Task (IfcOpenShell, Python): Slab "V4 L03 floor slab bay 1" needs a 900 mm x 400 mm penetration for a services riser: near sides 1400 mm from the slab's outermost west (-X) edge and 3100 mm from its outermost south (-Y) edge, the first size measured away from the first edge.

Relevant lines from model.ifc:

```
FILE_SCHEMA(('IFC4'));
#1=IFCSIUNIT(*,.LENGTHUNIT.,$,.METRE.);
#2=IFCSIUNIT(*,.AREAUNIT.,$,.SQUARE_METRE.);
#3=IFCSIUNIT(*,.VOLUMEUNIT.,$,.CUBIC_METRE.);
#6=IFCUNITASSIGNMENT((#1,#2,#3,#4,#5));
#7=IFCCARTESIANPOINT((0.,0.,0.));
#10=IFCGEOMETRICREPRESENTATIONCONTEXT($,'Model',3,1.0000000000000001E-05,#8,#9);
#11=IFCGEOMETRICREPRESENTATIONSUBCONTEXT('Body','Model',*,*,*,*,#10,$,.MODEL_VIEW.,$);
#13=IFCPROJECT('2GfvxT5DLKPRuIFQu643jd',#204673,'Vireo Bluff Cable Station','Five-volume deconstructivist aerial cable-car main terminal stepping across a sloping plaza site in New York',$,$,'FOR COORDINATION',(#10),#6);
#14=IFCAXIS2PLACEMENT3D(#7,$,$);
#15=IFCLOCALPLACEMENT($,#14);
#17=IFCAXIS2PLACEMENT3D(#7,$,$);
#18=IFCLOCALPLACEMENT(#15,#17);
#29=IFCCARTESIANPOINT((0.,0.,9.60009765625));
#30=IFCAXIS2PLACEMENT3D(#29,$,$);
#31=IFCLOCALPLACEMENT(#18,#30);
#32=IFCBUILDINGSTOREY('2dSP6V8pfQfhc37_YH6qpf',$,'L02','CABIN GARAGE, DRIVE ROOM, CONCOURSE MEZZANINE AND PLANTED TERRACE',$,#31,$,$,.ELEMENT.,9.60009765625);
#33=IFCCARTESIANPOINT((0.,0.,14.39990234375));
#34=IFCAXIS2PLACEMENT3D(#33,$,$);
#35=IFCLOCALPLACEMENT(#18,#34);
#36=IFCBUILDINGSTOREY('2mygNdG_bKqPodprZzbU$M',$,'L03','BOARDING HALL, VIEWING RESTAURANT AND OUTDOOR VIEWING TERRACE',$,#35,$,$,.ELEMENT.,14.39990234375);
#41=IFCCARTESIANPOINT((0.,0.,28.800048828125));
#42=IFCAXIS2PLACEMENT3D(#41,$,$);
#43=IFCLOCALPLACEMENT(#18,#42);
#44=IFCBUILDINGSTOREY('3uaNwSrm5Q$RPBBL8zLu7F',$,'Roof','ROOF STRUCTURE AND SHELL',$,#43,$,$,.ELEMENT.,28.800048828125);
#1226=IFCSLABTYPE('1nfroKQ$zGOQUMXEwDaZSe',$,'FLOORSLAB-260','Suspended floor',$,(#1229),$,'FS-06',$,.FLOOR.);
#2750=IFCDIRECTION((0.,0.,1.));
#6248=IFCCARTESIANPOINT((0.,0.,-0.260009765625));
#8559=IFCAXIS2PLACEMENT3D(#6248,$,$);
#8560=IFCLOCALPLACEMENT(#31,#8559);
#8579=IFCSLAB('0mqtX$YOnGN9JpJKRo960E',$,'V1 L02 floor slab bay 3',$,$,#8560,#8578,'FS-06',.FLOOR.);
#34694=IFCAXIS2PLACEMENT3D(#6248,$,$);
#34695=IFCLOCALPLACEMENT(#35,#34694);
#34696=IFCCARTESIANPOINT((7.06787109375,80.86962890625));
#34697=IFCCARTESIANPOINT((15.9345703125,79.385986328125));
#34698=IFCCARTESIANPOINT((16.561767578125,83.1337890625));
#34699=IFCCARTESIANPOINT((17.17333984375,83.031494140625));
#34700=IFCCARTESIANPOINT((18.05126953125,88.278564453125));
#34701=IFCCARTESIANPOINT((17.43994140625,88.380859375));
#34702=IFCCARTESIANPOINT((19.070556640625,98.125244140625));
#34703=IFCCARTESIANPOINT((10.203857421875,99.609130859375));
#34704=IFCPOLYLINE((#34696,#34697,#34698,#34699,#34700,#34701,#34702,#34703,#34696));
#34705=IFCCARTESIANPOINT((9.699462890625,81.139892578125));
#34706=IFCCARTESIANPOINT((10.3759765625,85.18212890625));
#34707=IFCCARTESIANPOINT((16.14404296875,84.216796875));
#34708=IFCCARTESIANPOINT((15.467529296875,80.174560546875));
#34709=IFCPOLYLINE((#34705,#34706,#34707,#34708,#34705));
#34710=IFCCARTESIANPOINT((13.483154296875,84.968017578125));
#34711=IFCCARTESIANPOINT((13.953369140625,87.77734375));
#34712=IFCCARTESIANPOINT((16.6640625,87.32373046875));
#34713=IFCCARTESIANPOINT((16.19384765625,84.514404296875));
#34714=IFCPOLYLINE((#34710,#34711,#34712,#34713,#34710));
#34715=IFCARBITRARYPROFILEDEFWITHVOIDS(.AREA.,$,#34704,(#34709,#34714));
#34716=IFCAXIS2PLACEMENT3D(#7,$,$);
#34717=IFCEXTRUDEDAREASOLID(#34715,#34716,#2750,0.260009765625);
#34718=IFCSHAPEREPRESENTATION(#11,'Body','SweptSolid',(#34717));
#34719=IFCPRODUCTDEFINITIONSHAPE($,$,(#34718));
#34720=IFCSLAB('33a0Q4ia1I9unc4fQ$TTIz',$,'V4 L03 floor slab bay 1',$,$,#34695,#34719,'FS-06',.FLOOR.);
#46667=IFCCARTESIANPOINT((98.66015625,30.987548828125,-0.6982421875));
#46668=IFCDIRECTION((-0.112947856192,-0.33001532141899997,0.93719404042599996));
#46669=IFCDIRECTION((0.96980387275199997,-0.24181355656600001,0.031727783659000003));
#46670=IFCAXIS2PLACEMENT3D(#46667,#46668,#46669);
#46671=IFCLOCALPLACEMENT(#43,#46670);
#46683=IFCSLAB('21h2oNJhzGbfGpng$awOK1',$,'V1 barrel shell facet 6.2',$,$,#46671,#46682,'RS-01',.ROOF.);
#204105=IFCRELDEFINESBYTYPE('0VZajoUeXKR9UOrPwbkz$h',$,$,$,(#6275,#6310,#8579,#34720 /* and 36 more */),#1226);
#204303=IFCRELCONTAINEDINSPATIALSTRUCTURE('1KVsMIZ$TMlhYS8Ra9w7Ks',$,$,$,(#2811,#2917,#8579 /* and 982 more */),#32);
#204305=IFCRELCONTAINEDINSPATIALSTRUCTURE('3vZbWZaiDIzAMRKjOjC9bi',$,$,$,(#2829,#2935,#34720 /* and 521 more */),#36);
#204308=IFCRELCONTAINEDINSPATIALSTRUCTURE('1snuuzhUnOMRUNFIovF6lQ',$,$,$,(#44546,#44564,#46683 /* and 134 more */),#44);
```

```python
import numpy as np
import ifcopenshell
import ifcopenshell.api.feature
import ifcopenshell.api.geometry
import ifcopenshell.api.root
import ifcopenshell.geom
import ifcopenshell.util.placement
import ifcopenshell.util.representation
import ifcopenshell.util.shape
import ifcopenshell.util.unit

model = ifcopenshell.open("model.ifc")
unit_scale = ifcopenshell.util.unit.calculate_unit_scale(model)
settings = ifcopenshell.geom.settings()


def volume(element):
    """Net volume in cubic metres, openings subtracted."""
    shape = ifcopenshell.geom.create_shape(settings, element)
    return ifcopenshell.util.shape.get_volume(shape.geometry)


slab = model.by_guid("33a0Q4ia1I9unc4fQ$TTIz")
before = volume(slab)

# Extent in the slab's own axes, in metres. The edges named are its -X and -Y sides.
slab_shape = ifcopenshell.geom.create_shape(settings, slab)
vertices = ifcopenshell.util.shape.get_vertices(slab_shape.geometry)
x_min, y_min, bottom = vertices.min(axis=0)
top = vertices[:, 2].max()

opening = ifcopenshell.api.root.create_entity(model, ifc_class="IfcOpeningElement", name="Services riser opening", predefined_type="OPENING")
context = ifcopenshell.util.representation.get_context(model, "Model", "Body", "MODEL_VIEW")
width, depth = 0.9, 0.4
outline = [(0.0, 0.0), (width, 0.0), (width, depth), (0.0, depth), (0.0, 0.0)]
# Overshoot both faces by 50 mm so the cut is clean.
shape = ifcopenshell.api.geometry.add_slab_representation(
    model, context=context, depth=top - bottom + 0.1, polyline=outline
)
ifcopenshell.api.geometry.assign_representation(model, product=opening, representation=shape)

matrix = ifcopenshell.util.placement.get_local_placement(slab.ObjectPlacement)
matrix[:, 3] = matrix @ np.append(np.array([x_min + 1.4, y_min + 3.1, bottom - 0.05]) / unit_scale, 1.0)
ifcopenshell.api.geometry.edit_object_placement(model, product=opening, matrix=matrix, is_si=False)
ifcopenshell.api.feature.add_feature(model, feature=opening, element=slab)

after = volume(slab)

print(f"slab volume {before:.3f} -> {after:.3f} m3")

model.write("model-out.ifc")
```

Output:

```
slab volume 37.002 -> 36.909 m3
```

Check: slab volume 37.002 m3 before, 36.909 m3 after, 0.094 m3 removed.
